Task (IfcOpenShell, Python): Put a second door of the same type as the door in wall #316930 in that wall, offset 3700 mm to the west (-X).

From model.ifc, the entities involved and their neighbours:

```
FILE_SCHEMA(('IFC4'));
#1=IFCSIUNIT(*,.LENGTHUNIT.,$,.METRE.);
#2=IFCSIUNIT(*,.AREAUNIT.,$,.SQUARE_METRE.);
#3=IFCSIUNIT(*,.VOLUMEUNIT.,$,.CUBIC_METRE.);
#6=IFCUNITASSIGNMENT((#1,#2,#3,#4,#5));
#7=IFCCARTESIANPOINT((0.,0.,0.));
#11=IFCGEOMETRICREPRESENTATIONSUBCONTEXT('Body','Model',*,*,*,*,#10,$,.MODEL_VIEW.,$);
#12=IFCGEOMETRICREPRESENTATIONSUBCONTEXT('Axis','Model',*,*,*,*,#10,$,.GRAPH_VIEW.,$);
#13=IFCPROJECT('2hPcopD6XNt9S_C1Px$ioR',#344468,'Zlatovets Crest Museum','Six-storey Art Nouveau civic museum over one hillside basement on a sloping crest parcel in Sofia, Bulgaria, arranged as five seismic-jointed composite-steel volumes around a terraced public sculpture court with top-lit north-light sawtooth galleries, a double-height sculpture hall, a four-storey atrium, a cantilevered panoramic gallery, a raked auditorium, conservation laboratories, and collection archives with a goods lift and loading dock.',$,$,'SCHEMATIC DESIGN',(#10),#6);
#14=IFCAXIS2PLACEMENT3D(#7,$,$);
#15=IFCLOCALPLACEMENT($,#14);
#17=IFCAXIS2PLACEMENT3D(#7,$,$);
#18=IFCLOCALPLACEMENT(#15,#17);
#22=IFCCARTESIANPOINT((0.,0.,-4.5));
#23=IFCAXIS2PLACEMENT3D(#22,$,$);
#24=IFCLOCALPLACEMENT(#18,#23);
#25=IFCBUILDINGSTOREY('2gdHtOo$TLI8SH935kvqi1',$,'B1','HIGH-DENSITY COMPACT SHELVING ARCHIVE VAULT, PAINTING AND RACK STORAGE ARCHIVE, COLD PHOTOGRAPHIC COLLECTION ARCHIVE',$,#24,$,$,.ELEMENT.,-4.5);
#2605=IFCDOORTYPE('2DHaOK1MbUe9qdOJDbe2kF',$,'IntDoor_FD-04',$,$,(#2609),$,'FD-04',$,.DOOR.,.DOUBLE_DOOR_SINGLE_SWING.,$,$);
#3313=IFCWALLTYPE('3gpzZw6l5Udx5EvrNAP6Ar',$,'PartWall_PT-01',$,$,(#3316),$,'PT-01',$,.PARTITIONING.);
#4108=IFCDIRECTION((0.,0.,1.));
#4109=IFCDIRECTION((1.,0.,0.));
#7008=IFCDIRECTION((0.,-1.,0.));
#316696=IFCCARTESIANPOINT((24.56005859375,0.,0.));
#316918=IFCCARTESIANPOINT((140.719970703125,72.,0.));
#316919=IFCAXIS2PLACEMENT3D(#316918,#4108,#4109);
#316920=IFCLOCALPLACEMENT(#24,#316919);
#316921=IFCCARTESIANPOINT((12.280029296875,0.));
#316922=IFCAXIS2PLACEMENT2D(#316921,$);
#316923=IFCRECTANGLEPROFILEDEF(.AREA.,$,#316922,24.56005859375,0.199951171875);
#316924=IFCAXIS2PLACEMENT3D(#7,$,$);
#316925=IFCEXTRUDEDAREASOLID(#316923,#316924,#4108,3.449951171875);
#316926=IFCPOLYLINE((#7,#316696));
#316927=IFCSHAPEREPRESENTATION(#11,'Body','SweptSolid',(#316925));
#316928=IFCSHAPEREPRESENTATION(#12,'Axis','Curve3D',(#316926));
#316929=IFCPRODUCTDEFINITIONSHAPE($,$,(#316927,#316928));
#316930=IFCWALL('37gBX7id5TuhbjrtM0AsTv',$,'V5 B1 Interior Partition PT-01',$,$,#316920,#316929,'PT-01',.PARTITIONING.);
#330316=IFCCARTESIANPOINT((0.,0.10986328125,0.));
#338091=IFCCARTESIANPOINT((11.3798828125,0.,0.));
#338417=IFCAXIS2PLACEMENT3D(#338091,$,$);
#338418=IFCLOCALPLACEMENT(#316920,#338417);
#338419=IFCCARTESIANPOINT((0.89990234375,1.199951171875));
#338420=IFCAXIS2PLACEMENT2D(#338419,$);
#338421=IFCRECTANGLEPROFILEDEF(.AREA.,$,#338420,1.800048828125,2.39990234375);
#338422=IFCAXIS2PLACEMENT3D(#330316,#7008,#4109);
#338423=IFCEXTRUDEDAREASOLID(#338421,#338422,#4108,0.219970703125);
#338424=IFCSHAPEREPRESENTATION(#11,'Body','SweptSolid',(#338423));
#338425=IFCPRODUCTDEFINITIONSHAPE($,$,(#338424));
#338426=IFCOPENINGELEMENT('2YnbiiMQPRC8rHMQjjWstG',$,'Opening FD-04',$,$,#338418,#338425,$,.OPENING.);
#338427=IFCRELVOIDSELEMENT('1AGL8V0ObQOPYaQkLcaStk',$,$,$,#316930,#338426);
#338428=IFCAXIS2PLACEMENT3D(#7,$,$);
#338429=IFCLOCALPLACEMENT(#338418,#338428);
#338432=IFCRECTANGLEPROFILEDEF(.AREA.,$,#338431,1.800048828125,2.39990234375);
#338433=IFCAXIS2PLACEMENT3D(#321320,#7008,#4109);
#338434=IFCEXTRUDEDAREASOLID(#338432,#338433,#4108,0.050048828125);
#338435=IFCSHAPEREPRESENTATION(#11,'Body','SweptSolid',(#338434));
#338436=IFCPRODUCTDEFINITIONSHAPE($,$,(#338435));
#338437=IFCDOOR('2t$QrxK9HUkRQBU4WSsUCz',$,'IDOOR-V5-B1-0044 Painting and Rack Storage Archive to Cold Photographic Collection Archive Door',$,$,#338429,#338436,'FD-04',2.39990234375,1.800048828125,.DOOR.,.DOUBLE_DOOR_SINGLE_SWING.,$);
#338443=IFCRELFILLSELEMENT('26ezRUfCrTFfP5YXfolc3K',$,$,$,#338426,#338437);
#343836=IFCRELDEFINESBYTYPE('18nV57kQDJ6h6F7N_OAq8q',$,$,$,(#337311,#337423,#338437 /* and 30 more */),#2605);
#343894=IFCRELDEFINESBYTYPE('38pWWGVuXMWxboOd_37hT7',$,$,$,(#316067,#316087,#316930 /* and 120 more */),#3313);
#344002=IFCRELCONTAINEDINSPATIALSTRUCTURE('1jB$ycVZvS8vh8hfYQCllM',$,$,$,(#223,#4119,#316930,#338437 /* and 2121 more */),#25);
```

```python
import ifcopenshell
import ifcopenshell.api.feature
import ifcopenshell.api.geometry
import ifcopenshell.api.root
import ifcopenshell.geom
import ifcopenshell.util.element
import ifcopenshell.util.placement
import ifcopenshell.util.shape
import ifcopenshell.util.unit

model = ifcopenshell.open("model.ifc")
unit_scale = ifcopenshell.util.unit.calculate_unit_scale(model)
settings = ifcopenshell.geom.settings()


def volume(element):
    """Net volume in cubic metres, openings subtracted."""
    shape = ifcopenshell.geom.create_shape(settings, element)
    return ifcopenshell.util.shape.get_volume(shape.geometry)


door = model.by_guid("2t$QrxK9HUkRQBU4WSsUCz")
opening = door.FillsVoids[0].RelatingOpeningElement
wall = opening.VoidsElements[0].RelatingBuildingElement
before = volume(wall)
shift = ifcopenshell.util.placement.get_local_placement(wall.ObjectPlacement)[:3, 0] * -3.7 / unit_scale

# copy_class copies the void relationship, type, container and properties, but no geometry.
new_opening = ifcopenshell.api.root.copy_class(model, product=opening)
new_opening.Representation = ifcopenshell.util.element.copy_deep(
    model, opening.Representation, exclude=["IfcGeometricRepresentationContext", "IfcRepresentationMap"]
)
new_door = ifcopenshell.api.root.copy_class(model, product=door)
new_door.Representation = ifcopenshell.util.element.copy_deep(
    model, door.Representation, exclude=["IfcGeometricRepresentationContext", "IfcRepresentationMap"]
)
new_door.Tag = None
ifcopenshell.api.feature.add_filling(model, opening=new_opening, element=new_door)

for old, new in ((opening, new_opening), (door, new_door)):
    matrix = ifcopenshell.util.placement.get_local_placement(old.ObjectPlacement)
    matrix[:3, 3] += shift
    ifcopenshell.api.geometry.edit_object_placement(model, product=new, matrix=matrix, is_si=False)

after = volume(wall)

print(f"wall volume {before:.3f} -> {after:.3f} m3")

model.write("model_v2.ifc")
```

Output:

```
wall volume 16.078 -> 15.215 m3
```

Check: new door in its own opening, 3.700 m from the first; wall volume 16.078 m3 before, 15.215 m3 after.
